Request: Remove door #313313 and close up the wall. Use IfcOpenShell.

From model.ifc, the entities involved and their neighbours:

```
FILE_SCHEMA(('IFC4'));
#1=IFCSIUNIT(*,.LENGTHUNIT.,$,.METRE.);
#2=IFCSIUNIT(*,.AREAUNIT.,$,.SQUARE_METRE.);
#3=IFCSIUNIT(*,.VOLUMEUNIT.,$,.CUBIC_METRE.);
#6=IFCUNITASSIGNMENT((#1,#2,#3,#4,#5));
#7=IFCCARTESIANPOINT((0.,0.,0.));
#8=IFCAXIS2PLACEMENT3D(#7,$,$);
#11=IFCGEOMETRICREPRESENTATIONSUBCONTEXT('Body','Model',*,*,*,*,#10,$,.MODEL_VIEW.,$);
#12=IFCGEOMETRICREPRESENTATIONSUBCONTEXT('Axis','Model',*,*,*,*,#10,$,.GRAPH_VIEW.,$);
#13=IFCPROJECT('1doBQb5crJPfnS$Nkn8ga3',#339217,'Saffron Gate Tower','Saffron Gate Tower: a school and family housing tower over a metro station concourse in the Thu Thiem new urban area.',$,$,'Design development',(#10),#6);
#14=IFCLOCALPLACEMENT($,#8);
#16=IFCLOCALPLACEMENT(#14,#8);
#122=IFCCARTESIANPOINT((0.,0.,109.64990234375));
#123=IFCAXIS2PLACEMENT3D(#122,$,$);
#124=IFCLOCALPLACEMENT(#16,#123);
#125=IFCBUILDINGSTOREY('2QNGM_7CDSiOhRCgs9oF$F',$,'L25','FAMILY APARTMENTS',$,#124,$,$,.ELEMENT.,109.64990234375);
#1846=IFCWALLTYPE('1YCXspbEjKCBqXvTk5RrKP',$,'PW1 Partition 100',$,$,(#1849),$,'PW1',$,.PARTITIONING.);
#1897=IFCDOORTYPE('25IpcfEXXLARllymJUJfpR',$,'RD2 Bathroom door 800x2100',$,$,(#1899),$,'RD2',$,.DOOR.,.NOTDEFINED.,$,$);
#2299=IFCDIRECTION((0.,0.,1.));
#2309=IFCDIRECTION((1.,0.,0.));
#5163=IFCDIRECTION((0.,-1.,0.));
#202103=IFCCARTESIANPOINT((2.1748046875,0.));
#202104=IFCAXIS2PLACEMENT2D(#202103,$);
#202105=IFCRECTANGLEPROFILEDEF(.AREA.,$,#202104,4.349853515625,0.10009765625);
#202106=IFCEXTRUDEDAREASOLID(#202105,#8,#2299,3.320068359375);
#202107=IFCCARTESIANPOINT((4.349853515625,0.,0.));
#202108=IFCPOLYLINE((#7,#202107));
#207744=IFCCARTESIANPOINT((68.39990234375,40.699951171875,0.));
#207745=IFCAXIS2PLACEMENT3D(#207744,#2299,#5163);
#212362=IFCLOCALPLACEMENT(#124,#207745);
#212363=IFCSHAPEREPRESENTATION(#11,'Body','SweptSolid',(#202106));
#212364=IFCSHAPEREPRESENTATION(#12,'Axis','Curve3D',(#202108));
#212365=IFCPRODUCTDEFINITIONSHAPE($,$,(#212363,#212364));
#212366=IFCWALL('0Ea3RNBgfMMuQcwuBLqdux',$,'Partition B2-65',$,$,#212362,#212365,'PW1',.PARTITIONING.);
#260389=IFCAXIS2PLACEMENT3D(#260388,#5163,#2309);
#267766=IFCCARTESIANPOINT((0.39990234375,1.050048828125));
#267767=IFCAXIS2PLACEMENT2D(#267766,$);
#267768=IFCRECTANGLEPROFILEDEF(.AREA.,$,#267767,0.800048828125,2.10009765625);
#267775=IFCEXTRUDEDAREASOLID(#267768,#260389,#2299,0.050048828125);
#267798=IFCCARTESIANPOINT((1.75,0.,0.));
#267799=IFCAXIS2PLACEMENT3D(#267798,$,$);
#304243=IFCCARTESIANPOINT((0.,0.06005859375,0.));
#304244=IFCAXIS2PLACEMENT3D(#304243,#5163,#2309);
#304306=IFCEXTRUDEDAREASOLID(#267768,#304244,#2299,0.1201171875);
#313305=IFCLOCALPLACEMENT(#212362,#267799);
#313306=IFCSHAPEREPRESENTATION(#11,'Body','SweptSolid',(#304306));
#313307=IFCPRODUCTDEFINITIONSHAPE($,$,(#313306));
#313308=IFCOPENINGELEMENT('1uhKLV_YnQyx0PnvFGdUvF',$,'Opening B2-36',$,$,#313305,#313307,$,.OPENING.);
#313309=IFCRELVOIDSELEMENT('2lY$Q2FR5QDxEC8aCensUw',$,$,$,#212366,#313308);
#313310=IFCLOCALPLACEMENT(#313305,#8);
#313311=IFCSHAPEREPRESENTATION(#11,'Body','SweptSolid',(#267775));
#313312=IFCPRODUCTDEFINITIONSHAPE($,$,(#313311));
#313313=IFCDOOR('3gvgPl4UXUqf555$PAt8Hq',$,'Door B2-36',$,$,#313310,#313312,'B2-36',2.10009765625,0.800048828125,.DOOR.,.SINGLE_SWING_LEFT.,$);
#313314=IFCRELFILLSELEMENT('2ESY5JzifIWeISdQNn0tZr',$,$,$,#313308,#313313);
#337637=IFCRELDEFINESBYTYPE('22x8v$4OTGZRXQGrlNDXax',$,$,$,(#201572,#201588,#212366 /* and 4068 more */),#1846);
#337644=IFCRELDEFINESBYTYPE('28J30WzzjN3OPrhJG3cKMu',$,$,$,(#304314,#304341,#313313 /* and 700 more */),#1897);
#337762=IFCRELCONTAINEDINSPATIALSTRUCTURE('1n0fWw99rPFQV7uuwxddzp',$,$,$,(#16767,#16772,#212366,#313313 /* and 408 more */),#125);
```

```python
import ifcopenshell
import ifcopenshell.api.feature
import ifcopenshell.api.root
import ifcopenshell.geom
import ifcopenshell.util.shape

model = ifcopenshell.open("model.ifc")
settings = ifcopenshell.geom.settings()


def volume(element):
    """Net volume in cubic metres, openings subtracted."""
    shape = ifcopenshell.geom.create_shape(settings, element)
    return ifcopenshell.util.shape.get_volume(shape.geometry)


door = model.by_guid("3gvgPl4UXUqf555$PAt8Hq")
opening = door.FillsVoids[0].RelatingOpeningElement
wall = opening.VoidsElements[0].RelatingBuildingElement
before = volume(wall)

ifcopenshell.api.root.remove_product(model, product=door)
ifcopenshell.api.feature.remove_feature(model, feature=opening)

after = volume(wall)

print(f"wall volume {before:.3f} -> {after:.3f} m3")

model.write("model_v2.ifc")
```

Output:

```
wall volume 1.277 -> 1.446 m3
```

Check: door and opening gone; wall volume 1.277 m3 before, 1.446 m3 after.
